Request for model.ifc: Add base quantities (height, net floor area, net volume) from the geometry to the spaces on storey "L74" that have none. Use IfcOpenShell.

First a look at what the model holds.

```python
import ifcopenshell
import ifcopenshell.util.element
import ifcopenshell.util.unit

model = ifcopenshell.open("model.ifc")
print(model.schema)
for unit_type in ("LENGTHUNIT", "AREAUNIT", "VOLUMEUNIT"):
    print(unit_type, ifcopenshell.util.unit.calculate_unit_scale(model, unit_type))
storey = next(s for s in model.by_type("IfcBuildingStorey") if s.Name == "L74")
spaces = [e for e in ifcopenshell.util.element.get_decomposition(storey) if e.is_a("IfcSpace")]
for e in sorted(spaces, key=lambda e: e.id()):
    print(e.id(), e.is_a(), e.Name, list(ifcopenshell.util.element.get_psets(e, qtos_only=True)), sep=" | ")
```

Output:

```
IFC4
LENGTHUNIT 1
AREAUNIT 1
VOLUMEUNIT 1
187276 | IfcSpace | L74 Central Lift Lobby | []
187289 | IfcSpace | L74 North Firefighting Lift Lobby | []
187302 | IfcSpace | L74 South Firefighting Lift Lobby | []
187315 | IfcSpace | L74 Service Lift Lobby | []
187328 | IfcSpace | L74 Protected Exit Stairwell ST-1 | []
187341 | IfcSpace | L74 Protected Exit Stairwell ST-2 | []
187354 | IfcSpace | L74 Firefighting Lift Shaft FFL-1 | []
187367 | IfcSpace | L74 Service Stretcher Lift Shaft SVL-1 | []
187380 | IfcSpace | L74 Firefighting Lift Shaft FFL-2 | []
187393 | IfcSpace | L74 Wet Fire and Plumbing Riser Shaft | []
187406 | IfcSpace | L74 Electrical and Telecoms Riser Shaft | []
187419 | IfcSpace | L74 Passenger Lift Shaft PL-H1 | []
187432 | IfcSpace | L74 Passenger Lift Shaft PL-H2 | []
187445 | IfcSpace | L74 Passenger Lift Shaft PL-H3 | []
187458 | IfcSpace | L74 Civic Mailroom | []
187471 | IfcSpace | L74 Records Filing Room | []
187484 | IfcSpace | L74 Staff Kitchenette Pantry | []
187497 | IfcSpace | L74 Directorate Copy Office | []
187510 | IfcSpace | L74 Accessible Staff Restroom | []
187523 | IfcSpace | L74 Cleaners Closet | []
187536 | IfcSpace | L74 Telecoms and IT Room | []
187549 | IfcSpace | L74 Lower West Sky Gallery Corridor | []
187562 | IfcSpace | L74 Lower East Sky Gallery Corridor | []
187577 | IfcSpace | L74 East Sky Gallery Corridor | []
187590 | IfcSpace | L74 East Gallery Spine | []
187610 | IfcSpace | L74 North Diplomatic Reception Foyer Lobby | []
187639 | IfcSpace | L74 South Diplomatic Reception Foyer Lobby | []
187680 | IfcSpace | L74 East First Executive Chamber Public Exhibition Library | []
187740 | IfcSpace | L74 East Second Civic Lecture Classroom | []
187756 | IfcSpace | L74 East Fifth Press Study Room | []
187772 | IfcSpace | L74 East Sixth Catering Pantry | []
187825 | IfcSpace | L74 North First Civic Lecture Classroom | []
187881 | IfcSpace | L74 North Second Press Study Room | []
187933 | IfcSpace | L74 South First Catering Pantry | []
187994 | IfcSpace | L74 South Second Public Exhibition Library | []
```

```python
import ifcopenshell
import ifcopenshell.api.pset
import ifcopenshell.geom
import ifcopenshell.util.element
import ifcopenshell.util.shape
import ifcopenshell.util.unit

model = ifcopenshell.open("model.ifc")
unit_scale = ifcopenshell.util.unit.calculate_unit_scale(model)
area_scale = ifcopenshell.util.unit.calculate_unit_scale(model, "AREAUNIT")
volume_scale = ifcopenshell.util.unit.calculate_unit_scale(model, "VOLUMEUNIT")
settings = ifcopenshell.geom.settings()

storey = next(s for s in model.by_type("IfcBuildingStorey") if s.Name == "L74")
spaces = [e for e in ifcopenshell.util.element.get_decomposition(storey) if e.is_a("IfcSpace")]

for e in sorted(spaces, key=lambda e: e.id()):
    if ifcopenshell.util.element.get_psets(e, qtos_only=True, should_inherit=False):
        continue
    # Geometry comes back in metres, in the element's own axes.
    shape = ifcopenshell.geom.create_shape(settings, e)
    values = {
        "Height": ifcopenshell.util.shape.get_z(shape.geometry) / unit_scale,
        "NetFloorArea": ifcopenshell.util.shape.get_footprint_area(shape.geometry) / area_scale,
        "NetVolume": ifcopenshell.util.shape.get_volume(shape.geometry) / volume_scale,
    }
    qto = ifcopenshell.api.pset.add_qto(model, product=e, name="Qto_SpaceBaseQuantities")
    ifcopenshell.api.pset.edit_qto(model, qto=qto, properties=values)
    print(e.id(), {k: round(v, 3) for k, v in values.items()})

model.write("model_v2.ifc")
```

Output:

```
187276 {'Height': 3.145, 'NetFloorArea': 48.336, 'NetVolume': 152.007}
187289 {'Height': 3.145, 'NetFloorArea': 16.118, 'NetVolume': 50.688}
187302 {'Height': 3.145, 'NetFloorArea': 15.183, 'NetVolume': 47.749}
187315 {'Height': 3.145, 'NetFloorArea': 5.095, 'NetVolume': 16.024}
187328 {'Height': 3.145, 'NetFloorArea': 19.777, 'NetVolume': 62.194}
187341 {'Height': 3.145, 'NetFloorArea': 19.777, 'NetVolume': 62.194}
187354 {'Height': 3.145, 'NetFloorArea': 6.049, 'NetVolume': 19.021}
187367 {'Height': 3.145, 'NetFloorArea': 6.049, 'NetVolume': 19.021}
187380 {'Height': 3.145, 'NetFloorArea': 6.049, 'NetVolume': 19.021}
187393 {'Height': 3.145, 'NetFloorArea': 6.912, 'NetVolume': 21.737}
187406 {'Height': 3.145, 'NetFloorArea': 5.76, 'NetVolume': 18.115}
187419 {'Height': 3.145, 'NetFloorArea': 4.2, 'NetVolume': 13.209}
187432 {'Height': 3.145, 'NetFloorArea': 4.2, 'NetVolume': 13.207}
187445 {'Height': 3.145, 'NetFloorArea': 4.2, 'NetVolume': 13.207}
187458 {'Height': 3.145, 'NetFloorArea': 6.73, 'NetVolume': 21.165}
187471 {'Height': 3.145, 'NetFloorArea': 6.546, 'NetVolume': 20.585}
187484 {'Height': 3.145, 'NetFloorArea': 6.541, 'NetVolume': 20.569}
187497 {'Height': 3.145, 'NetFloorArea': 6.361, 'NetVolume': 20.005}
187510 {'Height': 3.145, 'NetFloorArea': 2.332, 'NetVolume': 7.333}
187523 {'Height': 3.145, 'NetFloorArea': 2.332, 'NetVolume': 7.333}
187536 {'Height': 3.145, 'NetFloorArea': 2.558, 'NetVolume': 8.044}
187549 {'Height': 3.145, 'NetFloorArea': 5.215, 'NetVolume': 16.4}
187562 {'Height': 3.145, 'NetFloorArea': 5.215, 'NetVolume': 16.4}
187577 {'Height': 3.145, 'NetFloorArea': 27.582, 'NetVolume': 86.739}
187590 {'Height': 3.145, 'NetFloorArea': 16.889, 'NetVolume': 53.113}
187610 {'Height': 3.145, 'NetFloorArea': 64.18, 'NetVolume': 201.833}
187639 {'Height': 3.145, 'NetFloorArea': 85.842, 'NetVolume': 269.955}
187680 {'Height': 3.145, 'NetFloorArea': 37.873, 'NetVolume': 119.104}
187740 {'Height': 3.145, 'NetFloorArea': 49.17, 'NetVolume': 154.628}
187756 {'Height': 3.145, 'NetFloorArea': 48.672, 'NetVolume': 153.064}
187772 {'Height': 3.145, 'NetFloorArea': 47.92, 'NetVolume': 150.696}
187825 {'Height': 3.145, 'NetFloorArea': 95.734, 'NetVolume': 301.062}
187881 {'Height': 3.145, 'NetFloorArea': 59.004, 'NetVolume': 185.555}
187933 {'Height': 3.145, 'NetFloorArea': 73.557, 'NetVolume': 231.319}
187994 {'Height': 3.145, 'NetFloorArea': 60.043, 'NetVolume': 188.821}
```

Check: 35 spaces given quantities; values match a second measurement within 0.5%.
